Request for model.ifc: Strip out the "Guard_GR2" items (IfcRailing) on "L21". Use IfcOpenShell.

First a look at what the model holds.

```python
import ifcopenshell
import ifcopenshell.util.element

model = ifcopenshell.open("model.ifc")
print(model.schema)
storey = next(s for s in model.by_type("IfcBuildingStorey") if s.Name == "L21")
railings = [e for e in ifcopenshell.util.element.get_decomposition(storey) if e.is_a("IfcRailing")]
seen = {}
for e in railings:
    element_type = ifcopenshell.util.element.get_type(e)
    name = element_type.Name if element_type not in (None, e) else None
    seen[name] = seen.get(name, 0) + 1
for name, count in sorted(seen.items(), key=str):
    print(count, "x", name)
```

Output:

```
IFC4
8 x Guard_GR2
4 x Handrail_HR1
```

```python
import ifcopenshell
import ifcopenshell.api.root
import ifcopenshell.util.element

model = ifcopenshell.open("model.ifc")

storey = next(s for s in model.by_type("IfcBuildingStorey") if s.Name == "L21")
railings = [e for e in ifcopenshell.util.element.get_decomposition(storey) if e.is_a("IfcRailing")]
targets = [e for e in railings if (t := ifcopenshell.util.element.get_type(e)) not in (None, e) and t.Name == "Guard_GR2"]

for e in targets:
    ifcopenshell.api.root.remove_product(model, product=e)
print(len(targets), "removed")

model.write("model_edited.ifc")
```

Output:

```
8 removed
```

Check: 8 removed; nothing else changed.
